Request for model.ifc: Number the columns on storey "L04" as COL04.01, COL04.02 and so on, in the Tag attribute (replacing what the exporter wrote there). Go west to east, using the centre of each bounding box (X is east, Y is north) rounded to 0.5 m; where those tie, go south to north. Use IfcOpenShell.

First a look at what the model holds.

```python
import ifcopenshell
import ifcopenshell.util.element
import ifcopenshell.util.placement

model = ifcopenshell.open("model.ifc")
print(model.schema)
storey = next(s for s in model.by_type("IfcBuildingStorey") if s.Name == "L04")
columns = [e for e in ifcopenshell.util.element.get_decomposition(storey) if e.is_a("IfcColumn")]
for e in sorted(columns, key=lambda e: e.id()):
    origin = ifcopenshell.util.placement.get_local_placement(e.ObjectPlacement)[:3, 3]
    print(e.id(), e.Tag, e.Name, origin.round(2) + 0.0, sep=" | ")
```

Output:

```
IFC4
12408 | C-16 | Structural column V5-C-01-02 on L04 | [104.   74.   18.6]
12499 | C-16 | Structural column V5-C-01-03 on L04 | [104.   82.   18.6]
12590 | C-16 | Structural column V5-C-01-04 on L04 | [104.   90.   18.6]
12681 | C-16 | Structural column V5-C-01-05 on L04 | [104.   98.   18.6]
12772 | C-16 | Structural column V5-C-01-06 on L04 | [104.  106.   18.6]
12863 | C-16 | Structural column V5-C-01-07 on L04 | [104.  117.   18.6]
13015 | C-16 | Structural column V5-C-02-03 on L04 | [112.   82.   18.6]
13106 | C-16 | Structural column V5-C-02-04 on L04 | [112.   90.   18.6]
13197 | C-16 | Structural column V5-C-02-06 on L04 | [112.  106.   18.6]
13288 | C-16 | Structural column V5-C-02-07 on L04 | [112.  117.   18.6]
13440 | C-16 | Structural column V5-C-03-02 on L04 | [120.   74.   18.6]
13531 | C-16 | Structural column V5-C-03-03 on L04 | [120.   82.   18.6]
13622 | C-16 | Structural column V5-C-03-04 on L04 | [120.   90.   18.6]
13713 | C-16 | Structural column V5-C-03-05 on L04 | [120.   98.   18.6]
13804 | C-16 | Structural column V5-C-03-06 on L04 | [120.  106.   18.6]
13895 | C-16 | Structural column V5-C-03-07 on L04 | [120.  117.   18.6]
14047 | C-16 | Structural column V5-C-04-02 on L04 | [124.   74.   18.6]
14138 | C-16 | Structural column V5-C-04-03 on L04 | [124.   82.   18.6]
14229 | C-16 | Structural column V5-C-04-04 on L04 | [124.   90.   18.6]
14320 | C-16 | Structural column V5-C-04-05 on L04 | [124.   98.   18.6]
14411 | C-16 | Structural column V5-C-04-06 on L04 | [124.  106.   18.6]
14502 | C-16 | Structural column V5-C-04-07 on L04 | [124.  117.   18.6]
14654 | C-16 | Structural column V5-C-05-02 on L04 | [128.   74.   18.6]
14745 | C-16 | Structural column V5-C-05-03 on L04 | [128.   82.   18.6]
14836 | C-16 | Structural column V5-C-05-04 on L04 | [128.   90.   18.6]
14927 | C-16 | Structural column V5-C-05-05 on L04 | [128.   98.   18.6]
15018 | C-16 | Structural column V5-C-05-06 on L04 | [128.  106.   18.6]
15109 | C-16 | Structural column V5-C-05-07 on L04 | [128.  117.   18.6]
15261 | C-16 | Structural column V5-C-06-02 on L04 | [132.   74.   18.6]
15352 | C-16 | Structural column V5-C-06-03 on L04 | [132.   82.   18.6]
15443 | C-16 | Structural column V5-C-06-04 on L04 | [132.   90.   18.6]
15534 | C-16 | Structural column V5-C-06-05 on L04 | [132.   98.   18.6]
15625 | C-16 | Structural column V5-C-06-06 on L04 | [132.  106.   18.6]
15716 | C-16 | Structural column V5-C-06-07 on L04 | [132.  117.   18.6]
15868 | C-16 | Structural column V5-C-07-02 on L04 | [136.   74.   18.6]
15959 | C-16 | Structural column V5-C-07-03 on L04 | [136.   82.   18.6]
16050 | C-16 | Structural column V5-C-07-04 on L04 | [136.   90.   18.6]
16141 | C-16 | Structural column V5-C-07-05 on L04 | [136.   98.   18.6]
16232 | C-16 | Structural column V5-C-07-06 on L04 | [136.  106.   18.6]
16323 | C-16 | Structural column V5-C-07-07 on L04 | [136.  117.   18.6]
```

```python
import ifcopenshell
import ifcopenshell.geom
import ifcopenshell.util.element
import ifcopenshell.util.shape

model = ifcopenshell.open("model.ifc")
settings = ifcopenshell.geom.settings()
settings.set("use-world-coords", True)


def centre(element):
    shape = ifcopenshell.geom.create_shape(settings, element)
    return ifcopenshell.util.shape.get_bbox_centroid(shape.geometry)


storey = next(s for s in model.by_type("IfcBuildingStorey") if s.Name == "L04")
columns = [e for e in ifcopenshell.util.element.get_decomposition(storey) if e.is_a("IfcColumn")]

# Insertion points can sit at a corner or the storey origin, so sort by the geometry (in metres).
centres = {e: centre(e) for e in columns}
columns.sort(key=lambda e: (round(centres[e][0] / 0.5), centres[e][1]))

for i, e in enumerate(columns, start=1):
    number = f"COL04.{i:02d}"
    e.Tag = number
    print(e.id(), number)

model.write("model_edited.ifc")
```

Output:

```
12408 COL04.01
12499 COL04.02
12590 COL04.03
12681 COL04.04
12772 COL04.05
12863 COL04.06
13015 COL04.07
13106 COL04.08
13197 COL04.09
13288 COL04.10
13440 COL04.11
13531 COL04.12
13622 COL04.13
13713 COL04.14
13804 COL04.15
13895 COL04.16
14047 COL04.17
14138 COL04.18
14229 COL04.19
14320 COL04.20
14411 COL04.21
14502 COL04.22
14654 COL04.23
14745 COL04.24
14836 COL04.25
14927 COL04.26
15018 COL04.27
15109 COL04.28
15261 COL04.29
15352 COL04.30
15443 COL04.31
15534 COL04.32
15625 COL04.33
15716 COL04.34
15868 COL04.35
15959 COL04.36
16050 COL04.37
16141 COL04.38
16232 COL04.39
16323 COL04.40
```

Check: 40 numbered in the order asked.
